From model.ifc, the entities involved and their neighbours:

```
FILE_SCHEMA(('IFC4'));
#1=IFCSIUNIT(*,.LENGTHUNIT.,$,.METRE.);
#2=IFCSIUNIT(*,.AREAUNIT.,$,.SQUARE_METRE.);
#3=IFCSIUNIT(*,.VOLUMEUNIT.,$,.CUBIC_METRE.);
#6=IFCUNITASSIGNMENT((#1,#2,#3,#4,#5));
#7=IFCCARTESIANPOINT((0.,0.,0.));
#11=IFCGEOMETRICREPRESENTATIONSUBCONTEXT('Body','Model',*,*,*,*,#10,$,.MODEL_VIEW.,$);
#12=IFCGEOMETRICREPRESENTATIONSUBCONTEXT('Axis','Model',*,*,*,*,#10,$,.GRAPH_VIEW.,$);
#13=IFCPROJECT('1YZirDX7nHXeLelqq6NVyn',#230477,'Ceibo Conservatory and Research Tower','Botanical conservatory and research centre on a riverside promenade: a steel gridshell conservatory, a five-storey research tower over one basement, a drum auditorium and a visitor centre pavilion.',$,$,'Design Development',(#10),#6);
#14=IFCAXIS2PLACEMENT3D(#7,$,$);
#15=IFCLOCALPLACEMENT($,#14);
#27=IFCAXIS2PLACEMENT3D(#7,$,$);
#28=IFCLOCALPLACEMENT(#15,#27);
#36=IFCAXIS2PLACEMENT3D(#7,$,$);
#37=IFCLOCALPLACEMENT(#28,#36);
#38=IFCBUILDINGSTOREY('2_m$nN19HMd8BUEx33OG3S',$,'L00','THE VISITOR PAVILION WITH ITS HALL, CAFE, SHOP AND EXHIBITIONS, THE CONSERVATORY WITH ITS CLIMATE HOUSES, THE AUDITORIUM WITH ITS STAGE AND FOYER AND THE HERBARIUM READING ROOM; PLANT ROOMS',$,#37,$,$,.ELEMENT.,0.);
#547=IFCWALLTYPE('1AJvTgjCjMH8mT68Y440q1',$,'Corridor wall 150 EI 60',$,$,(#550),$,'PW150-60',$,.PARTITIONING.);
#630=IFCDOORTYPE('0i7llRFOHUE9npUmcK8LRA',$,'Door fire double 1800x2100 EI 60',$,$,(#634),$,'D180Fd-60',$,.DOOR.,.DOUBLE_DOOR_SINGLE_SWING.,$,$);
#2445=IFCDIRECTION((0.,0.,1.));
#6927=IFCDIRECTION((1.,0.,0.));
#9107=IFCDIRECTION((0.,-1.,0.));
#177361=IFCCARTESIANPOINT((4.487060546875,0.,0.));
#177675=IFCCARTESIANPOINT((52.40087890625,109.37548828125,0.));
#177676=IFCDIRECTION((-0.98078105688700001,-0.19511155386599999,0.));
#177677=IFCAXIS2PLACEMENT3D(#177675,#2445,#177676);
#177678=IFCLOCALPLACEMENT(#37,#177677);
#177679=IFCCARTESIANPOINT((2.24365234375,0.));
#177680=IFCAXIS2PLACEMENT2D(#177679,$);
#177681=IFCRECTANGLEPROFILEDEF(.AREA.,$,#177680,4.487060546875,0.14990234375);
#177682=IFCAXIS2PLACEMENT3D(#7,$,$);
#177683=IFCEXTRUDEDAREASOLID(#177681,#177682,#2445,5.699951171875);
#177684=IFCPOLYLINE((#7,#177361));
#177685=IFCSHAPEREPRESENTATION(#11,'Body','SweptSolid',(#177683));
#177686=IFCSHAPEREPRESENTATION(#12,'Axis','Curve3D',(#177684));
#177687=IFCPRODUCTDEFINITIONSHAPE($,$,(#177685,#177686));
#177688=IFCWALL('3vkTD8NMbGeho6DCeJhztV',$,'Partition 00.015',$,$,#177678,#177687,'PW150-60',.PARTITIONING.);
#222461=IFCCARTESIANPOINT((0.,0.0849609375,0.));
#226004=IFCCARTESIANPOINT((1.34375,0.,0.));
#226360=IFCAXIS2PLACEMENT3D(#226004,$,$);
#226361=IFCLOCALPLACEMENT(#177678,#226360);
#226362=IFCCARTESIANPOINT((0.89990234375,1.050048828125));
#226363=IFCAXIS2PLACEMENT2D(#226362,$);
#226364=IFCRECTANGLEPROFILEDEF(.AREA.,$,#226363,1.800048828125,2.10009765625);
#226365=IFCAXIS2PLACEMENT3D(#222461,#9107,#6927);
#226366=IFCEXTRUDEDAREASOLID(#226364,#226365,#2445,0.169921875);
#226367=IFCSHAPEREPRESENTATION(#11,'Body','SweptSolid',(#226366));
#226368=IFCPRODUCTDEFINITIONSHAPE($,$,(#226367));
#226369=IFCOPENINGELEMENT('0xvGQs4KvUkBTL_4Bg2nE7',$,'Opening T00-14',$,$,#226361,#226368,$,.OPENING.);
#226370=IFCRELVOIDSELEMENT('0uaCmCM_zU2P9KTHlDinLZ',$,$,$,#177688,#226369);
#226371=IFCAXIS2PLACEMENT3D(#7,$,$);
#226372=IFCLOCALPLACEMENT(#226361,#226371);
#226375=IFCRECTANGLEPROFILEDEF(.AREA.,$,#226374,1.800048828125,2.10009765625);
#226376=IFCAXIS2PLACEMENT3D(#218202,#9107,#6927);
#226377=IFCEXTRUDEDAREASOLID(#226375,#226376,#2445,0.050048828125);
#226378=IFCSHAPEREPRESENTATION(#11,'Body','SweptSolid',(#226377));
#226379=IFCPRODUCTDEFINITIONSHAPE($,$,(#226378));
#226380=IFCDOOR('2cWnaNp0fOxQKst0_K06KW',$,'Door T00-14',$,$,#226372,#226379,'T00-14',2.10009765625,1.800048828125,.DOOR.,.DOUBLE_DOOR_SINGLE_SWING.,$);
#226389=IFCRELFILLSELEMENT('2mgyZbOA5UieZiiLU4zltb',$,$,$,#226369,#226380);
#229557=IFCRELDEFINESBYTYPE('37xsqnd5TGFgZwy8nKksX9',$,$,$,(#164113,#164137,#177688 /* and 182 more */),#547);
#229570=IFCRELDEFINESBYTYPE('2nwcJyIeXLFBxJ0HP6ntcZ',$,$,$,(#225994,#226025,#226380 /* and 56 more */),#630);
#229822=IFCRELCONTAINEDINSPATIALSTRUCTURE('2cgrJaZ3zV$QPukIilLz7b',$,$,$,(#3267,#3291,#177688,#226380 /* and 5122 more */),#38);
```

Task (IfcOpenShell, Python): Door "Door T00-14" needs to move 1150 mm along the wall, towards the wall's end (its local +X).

```python
import ifcopenshell
import ifcopenshell.api.geometry
import ifcopenshell.util.placement
import ifcopenshell.util.unit

model = ifcopenshell.open("model.ifc")
unit_scale = ifcopenshell.util.unit.calculate_unit_scale(model)

door = model.by_guid("2cWnaNp0fOxQKst0_K06KW")
opening = door.FillsVoids[0].RelatingOpeningElement
wall = opening.VoidsElements[0].RelatingBuildingElement

wall_matrix = ifcopenshell.util.placement.get_local_placement(wall.ObjectPlacement)
shift = wall_matrix[:3, 0] * 1.15 / unit_scale
before = ifcopenshell.util.placement.get_local_placement(door.ObjectPlacement)[:3, 3].copy()

# The door is placed relative to its opening, so it follows when the opening moves.
matrix = ifcopenshell.util.placement.get_local_placement(opening.ObjectPlacement)
matrix[:3, 3] += shift
ifcopenshell.api.geometry.edit_object_placement(
    model, product=opening, matrix=matrix, is_si=False, should_transform_children=True
)

after = ifcopenshell.util.placement.get_local_placement(door.ObjectPlacement)[:3, 3]
print("door moved by", (after - before).round(3) + 0.0)

model.write("model_v2.ifc")
```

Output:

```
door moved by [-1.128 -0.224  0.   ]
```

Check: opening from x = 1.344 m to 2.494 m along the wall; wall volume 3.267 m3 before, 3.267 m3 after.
